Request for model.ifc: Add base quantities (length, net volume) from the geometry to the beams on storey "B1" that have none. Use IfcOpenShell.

First a look at what the model holds.

```python
import ifcopenshell
import ifcopenshell.util.element
import ifcopenshell.util.unit

model = ifcopenshell.open("model.ifc")
print(model.schema)
for unit_type in ("LENGTHUNIT", "AREAUNIT", "VOLUMEUNIT"):
    print(unit_type, ifcopenshell.util.unit.calculate_unit_scale(model, unit_type))
storey = next(s for s in model.by_type("IfcBuildingStorey") if s.Name == "B1")
beams = [e for e in ifcopenshell.util.element.get_decomposition(storey) if e.is_a("IfcBeam")]
for e in sorted(beams, key=lambda e: e.id()):
    print(e.id(), e.is_a(), e.Name, list(ifcopenshell.util.element.get_psets(e, qtos_only=True)), sep=" | ")
```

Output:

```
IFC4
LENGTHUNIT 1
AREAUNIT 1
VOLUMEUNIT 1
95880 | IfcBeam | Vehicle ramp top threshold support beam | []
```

```python
import ifcopenshell
import ifcopenshell.api.pset
import ifcopenshell.geom
import ifcopenshell.util.element
import ifcopenshell.util.shape
import ifcopenshell.util.unit

model = ifcopenshell.open("model.ifc")
unit_scale = ifcopenshell.util.unit.calculate_unit_scale(model)
volume_scale = ifcopenshell.util.unit.calculate_unit_scale(model, "VOLUMEUNIT")
settings = ifcopenshell.geom.settings()

storey = next(s for s in model.by_type("IfcBuildingStorey") if s.Name == "B1")
beams = [e for e in ifcopenshell.util.element.get_decomposition(storey) if e.is_a("IfcBeam")]

for e in sorted(beams, key=lambda e: e.id()):
    if ifcopenshell.util.element.get_psets(e, qtos_only=True, should_inherit=False):
        continue
    # Geometry comes back in metres, in the element's own axes.
    shape = ifcopenshell.geom.create_shape(settings, e)
    values = {
        "Length": ifcopenshell.util.shape.get_max_xyz(shape.geometry) / unit_scale,
        "NetVolume": ifcopenshell.util.shape.get_volume(shape.geometry) / volume_scale,
    }
    qto = ifcopenshell.api.pset.add_qto(model, product=e, name="Qto_BeamBaseQuantities")
    ifcopenshell.api.pset.edit_qto(model, qto=qto, properties=values)
    print(e.id(), {k: round(v, 3) for k, v in values.items()})

model.write("model_edited.ifc")
```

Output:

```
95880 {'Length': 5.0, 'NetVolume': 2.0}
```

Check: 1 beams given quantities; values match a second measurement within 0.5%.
